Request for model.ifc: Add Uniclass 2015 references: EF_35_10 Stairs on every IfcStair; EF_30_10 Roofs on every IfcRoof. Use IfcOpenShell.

First a look at what the model holds.

```python
import ifcopenshell

model = ifcopenshell.open("model.ifc")
print(model.schema)
print("classifications:", [c.Name for c in model.by_type("IfcClassification")])
for ifc_class in ("IfcDoor", "IfcRoof", "IfcStair", "IfcWall", "IfcWindow"):
    print(ifc_class, len(model.by_type(ifc_class)))
```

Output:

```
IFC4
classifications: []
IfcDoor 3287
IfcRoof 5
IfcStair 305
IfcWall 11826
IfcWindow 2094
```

```python
import ifcopenshell
import ifcopenshell.api.classification

model = ifcopenshell.open("model.ifc")

system = ifcopenshell.api.classification.add_classification(model, classification="Uniclass 2015")

codes = {
    "IfcStair": ("EF_35_10", "Stairs"),
    "IfcRoof": ("EF_30_10", "Roofs"),
}
for ifc_class, (code, name) in codes.items():
    products = model.by_type(ifc_class)
    ifcopenshell.api.classification.add_reference(
        model, products=products, classification=system, identification=code, name=name
    )
    print(code, len(products))

model.write("model_rev.ifc")
```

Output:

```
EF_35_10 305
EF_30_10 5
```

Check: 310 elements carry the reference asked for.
